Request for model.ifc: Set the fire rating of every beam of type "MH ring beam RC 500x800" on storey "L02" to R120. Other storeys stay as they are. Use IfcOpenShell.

First a look at what the model holds.

```python
import ifcopenshell
import ifcopenshell.util.element

model = ifcopenshell.open("model.ifc")
print(model.schema)
storey = next(s for s in model.by_type("IfcBuildingStorey") if s.Name == "L02")
beams = [e for e in ifcopenshell.util.element.get_decomposition(storey) if e.is_a("IfcBeam")]
seen = {}
for e in beams:
    element_type = ifcopenshell.util.element.get_type(e)
    key = (element_type.Name if element_type != e and element_type else None, ifcopenshell.util.element.get_pset(e, "Pset_BeamCommon", "FireRating"))
    seen[key] = seen.get(key, 0) + 1
for (name, value), count in sorted(seen.items(), key=str):
    print(count, "x", name, "|", value)
```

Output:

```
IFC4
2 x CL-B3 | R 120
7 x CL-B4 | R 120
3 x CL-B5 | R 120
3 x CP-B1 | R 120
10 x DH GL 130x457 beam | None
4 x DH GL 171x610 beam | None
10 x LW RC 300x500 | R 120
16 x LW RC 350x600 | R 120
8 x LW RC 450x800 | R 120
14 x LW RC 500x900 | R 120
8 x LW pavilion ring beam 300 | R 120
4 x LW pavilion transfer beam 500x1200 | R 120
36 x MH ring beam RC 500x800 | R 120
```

```python
import ifcopenshell
import ifcopenshell.api.pset
import ifcopenshell.util.element

model = ifcopenshell.open("model.ifc")

storey = next(s for s in model.by_type("IfcBuildingStorey") if s.Name == "L02")
beams = [e for e in ifcopenshell.util.element.get_decomposition(storey) if e.is_a("IfcBeam")]

count = 0
for e in beams:
    element_type = ifcopenshell.util.element.get_type(e)
    if element_type in (None, e) or element_type.Name != "MH ring beam RC 500x800":
        continue
    # add_pset returns the element's existing set when there is one.
    pset = ifcopenshell.api.pset.add_pset(model, product=e, name="Pset_BeamCommon")
    ifcopenshell.api.pset.edit_pset(model, pset=pset, properties={"FireRating": "R120"})
    count += 1

print(count, "beams updated")

model.write("model-out.ifc")
```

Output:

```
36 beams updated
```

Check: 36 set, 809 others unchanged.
